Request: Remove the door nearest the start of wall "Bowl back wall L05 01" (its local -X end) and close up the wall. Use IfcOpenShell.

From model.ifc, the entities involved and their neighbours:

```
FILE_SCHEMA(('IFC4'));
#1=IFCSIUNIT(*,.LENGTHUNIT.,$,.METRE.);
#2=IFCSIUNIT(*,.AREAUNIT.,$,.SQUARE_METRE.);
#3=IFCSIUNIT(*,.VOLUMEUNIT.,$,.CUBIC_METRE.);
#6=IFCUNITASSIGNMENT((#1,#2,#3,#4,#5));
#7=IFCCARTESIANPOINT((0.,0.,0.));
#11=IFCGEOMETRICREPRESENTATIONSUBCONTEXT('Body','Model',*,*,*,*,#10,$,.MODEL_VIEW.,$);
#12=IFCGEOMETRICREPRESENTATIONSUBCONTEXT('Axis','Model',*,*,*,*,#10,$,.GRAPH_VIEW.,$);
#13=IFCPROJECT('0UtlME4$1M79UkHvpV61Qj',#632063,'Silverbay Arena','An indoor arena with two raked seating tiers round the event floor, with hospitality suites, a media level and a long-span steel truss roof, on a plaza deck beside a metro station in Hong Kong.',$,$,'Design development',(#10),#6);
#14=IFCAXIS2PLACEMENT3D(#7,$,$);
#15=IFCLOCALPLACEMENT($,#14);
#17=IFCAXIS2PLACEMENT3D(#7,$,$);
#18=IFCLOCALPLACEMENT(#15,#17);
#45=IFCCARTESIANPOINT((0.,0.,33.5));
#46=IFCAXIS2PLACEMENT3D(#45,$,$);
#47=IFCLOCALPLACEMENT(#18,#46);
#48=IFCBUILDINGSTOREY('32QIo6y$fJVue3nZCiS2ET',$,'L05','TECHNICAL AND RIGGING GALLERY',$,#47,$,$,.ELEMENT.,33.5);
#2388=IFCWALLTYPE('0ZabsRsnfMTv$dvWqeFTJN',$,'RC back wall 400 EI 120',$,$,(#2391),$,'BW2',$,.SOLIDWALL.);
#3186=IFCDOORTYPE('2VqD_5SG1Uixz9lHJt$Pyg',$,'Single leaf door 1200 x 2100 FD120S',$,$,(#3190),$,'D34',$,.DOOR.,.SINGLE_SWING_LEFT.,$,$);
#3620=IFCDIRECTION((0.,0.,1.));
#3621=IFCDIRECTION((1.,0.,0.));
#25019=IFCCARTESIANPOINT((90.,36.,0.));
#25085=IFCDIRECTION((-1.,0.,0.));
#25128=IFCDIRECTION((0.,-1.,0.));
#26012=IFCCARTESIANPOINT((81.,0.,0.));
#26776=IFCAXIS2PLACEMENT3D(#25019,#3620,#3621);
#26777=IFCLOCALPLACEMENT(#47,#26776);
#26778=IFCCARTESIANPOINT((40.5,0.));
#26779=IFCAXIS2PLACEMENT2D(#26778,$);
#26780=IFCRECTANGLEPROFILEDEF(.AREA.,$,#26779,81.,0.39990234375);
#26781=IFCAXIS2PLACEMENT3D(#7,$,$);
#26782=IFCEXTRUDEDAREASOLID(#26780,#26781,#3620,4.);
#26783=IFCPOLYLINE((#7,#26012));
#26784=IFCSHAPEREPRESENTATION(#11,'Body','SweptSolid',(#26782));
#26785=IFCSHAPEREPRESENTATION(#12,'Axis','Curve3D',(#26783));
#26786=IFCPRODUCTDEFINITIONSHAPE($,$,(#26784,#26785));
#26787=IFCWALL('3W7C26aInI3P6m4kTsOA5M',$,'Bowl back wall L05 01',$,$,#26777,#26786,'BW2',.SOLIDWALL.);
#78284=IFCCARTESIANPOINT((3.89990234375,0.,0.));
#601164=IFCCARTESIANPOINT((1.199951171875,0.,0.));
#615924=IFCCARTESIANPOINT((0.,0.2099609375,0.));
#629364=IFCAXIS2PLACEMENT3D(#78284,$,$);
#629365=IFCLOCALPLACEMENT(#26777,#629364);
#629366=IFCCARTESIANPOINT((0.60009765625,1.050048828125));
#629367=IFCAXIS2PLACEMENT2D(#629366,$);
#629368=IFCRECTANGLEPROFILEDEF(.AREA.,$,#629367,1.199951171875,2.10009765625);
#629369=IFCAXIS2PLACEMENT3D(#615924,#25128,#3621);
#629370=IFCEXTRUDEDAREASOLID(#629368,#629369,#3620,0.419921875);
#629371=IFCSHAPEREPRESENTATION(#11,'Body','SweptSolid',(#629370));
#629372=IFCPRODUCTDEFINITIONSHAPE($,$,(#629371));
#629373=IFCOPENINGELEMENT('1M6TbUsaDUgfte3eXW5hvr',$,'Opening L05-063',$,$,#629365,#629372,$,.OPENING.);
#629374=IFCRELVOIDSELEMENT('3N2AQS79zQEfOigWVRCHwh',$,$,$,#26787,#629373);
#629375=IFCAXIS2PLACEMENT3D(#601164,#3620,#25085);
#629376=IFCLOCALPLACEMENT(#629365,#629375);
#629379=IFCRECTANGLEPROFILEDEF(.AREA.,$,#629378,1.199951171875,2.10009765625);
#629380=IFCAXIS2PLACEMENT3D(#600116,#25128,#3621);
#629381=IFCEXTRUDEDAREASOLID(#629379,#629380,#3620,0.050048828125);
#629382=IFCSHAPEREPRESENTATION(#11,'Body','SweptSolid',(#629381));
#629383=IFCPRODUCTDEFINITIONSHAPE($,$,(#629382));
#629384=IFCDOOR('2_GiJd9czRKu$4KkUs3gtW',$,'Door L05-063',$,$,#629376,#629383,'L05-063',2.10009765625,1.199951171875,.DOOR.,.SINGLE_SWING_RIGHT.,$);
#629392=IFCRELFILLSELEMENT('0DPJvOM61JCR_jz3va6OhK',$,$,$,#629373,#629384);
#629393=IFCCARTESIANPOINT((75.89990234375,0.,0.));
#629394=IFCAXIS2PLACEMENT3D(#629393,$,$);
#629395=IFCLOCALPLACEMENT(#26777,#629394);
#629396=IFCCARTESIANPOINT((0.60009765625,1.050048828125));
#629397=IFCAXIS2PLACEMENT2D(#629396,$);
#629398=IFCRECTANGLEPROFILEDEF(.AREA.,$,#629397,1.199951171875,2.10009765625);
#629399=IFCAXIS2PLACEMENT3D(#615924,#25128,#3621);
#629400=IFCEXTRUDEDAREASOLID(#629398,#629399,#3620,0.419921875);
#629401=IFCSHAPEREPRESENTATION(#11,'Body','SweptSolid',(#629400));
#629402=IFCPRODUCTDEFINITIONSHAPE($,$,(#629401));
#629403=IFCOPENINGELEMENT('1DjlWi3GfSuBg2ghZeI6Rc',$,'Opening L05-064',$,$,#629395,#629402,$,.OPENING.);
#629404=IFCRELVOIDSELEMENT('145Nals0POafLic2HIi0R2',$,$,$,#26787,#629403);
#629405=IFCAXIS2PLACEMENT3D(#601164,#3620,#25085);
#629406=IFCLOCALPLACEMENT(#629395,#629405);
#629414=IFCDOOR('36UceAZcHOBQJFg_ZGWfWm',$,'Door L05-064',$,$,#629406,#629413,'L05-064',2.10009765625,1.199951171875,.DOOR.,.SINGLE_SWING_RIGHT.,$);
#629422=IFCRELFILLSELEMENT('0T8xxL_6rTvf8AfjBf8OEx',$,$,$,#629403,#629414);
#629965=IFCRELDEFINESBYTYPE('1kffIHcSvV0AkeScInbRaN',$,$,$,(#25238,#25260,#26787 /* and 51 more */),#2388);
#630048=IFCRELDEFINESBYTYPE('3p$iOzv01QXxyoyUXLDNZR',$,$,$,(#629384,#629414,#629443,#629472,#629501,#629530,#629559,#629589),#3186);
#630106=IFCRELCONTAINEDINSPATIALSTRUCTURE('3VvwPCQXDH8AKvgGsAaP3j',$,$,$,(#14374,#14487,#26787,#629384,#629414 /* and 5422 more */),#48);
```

```python
import ifcopenshell
import ifcopenshell.api.feature
import ifcopenshell.api.root
import ifcopenshell.geom
import ifcopenshell.util.shape

model = ifcopenshell.open("model.ifc")
settings = ifcopenshell.geom.settings()


def volume(element):
    """Net volume in cubic metres, openings subtracted."""
    shape = ifcopenshell.geom.create_shape(settings, element)
    return ifcopenshell.util.shape.get_volume(shape.geometry)


door = model.by_guid("2_GiJd9czRKu$4KkUs3gtW")
opening = door.FillsVoids[0].RelatingOpeningElement
wall = opening.VoidsElements[0].RelatingBuildingElement
before = volume(wall)

ifcopenshell.api.root.remove_product(model, product=door)
ifcopenshell.api.feature.remove_feature(model, feature=opening)

after = volume(wall)

print(f"wall volume {before:.3f} -> {after:.3f} m3")

model.write("model_updated.ifc")
```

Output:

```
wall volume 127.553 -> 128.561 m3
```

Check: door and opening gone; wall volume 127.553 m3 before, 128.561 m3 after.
